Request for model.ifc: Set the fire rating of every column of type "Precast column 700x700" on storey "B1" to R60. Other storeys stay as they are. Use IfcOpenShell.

First a look at what the model holds.

```python
import ifcopenshell
import ifcopenshell.util.element

model = ifcopenshell.open("model.ifc")
print(model.schema)
storey = next(s for s in model.by_type("IfcBuildingStorey") if s.Name == "B1")
columns = [e for e in ifcopenshell.util.element.get_decomposition(storey) if e.is_a("IfcColumn")]
seen = {}
for e in columns:
    element_type = ifcopenshell.util.element.get_type(e)
    key = (element_type.Name if element_type != e and element_type else None, ifcopenshell.util.element.get_pset(e, "Pset_ColumnCommon", "FireRating"))
    seen[key] = seen.get(key, 0) + 1
for (name, value), count in sorted(seen.items(), key=str):
    print(count, "x", name, "|", value)
```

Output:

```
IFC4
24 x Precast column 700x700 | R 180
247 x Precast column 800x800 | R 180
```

```python
import ifcopenshell
import ifcopenshell.api.pset
import ifcopenshell.util.element

model = ifcopenshell.open("model.ifc")

storey = next(s for s in model.by_type("IfcBuildingStorey") if s.Name == "B1")
columns = [e for e in ifcopenshell.util.element.get_decomposition(storey) if e.is_a("IfcColumn")]

count = 0
for e in columns:
    element_type = ifcopenshell.util.element.get_type(e)
    if element_type in (None, e) or element_type.Name != "Precast column 700x700":
        continue
    # add_pset returns the element's existing set when there is one.
    pset = ifcopenshell.api.pset.add_pset(model, product=e, name="Pset_ColumnCommon")
    ifcopenshell.api.pset.edit_pset(model, pset=pset, properties={"FireRating": "R60"})
    count += 1

print(count, "columns updated")

model.write("model_v2.ifc")
```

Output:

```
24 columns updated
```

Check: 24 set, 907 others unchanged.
